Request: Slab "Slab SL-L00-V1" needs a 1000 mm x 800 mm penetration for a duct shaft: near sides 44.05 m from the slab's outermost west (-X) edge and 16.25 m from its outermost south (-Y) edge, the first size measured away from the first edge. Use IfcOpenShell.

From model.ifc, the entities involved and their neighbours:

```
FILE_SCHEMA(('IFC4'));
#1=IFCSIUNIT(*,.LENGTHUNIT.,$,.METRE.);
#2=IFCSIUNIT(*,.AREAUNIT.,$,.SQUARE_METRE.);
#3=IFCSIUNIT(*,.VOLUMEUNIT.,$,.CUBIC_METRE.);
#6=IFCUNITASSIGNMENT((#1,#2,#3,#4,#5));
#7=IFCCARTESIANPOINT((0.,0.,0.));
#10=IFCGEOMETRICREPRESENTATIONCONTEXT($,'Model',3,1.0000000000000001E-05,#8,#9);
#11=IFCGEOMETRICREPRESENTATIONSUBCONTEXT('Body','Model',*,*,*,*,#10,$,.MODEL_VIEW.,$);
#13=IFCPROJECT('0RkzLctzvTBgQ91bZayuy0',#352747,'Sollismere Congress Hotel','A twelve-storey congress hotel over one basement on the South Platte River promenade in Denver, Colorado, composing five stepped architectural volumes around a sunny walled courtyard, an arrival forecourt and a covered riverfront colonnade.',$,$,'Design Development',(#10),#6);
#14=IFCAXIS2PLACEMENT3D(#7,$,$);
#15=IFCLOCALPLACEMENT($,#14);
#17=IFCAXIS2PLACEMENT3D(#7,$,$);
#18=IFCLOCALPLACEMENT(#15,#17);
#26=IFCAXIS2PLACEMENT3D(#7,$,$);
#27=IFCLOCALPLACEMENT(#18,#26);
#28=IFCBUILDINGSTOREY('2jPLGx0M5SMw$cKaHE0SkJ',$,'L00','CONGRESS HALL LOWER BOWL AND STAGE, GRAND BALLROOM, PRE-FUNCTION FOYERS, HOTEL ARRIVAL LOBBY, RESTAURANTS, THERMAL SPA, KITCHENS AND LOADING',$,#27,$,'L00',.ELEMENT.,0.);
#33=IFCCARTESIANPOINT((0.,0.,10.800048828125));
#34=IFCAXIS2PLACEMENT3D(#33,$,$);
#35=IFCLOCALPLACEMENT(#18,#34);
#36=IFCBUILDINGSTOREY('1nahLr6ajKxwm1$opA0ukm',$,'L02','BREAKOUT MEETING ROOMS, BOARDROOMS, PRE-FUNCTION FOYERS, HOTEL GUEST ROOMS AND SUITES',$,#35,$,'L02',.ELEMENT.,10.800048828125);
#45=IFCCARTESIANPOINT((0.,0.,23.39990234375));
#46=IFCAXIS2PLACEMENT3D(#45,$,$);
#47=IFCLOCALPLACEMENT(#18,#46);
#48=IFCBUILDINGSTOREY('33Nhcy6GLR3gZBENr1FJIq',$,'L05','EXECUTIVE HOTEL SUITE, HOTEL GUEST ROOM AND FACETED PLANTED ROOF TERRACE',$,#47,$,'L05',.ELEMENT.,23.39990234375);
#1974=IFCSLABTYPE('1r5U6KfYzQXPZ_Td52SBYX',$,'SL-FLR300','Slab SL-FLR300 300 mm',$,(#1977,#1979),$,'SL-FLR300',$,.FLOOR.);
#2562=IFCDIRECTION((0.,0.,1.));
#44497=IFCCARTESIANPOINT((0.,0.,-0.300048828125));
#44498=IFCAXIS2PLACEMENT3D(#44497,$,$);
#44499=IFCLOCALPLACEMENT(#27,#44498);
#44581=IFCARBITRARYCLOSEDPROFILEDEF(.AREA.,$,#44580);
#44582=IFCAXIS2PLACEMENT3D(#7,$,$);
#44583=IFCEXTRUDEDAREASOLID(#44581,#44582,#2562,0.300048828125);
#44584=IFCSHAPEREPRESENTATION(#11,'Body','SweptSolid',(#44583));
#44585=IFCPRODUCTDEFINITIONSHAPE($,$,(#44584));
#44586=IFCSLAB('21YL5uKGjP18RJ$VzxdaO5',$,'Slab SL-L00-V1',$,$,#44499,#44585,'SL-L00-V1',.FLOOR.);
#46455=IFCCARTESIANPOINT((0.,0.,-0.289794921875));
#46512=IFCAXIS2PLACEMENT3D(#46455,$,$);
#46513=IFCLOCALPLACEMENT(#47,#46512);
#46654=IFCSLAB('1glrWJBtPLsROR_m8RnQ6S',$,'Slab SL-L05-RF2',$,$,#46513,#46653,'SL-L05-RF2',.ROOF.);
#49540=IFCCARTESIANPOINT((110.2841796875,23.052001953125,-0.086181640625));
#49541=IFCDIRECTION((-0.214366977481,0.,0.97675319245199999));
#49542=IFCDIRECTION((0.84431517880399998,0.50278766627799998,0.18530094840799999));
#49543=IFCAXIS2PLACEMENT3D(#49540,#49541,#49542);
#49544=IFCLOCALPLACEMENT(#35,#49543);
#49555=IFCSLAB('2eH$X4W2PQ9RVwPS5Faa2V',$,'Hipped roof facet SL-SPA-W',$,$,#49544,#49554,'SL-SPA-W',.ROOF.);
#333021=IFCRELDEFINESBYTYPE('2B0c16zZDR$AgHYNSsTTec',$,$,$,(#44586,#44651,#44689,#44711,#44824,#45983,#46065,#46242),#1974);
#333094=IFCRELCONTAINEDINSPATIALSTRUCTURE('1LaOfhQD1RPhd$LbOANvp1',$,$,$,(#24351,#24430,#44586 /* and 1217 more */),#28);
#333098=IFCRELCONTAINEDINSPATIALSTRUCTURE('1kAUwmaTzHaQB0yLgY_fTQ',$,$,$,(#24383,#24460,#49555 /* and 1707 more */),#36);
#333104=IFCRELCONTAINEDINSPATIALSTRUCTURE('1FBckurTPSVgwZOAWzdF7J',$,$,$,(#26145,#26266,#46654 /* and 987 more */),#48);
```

```python
import numpy as np
import ifcopenshell
import ifcopenshell.api.feature
import ifcopenshell.api.geometry
import ifcopenshell.api.root
import ifcopenshell.geom
import ifcopenshell.util.placement
import ifcopenshell.util.representation
import ifcopenshell.util.shape
import ifcopenshell.util.unit

model = ifcopenshell.open("model.ifc")
unit_scale = ifcopenshell.util.unit.calculate_unit_scale(model)
settings = ifcopenshell.geom.settings()


def volume(element):
    """Net volume in cubic metres, openings subtracted."""
    shape = ifcopenshell.geom.create_shape(settings, element)
    return ifcopenshell.util.shape.get_volume(shape.geometry)


slab = model.by_guid("21YL5uKGjP18RJ$VzxdaO5")
before = volume(slab)

# Extent in the slab's own axes, in metres. The edges named are its -X and -Y sides.
slab_shape = ifcopenshell.geom.create_shape(settings, slab)
vertices = ifcopenshell.util.shape.get_vertices(slab_shape.geometry)
x_min, y_min, bottom = vertices.min(axis=0)
top = vertices[:, 2].max()

opening = ifcopenshell.api.root.create_entity(model, ifc_class="IfcOpeningElement", name="Duct shaft opening", predefined_type="OPENING")
context = ifcopenshell.util.representation.get_context(model, "Model", "Body", "MODEL_VIEW")
width, depth = 1, 0.8
outline = [(0.0, 0.0), (width, 0.0), (width, depth), (0.0, depth), (0.0, 0.0)]
# Overshoot both faces by 50 mm so the cut is clean.
shape = ifcopenshell.api.geometry.add_slab_representation(
    model, context=context, depth=top - bottom + 0.1, polyline=outline
)
ifcopenshell.api.geometry.assign_representation(model, product=opening, representation=shape)

matrix = ifcopenshell.util.placement.get_local_placement(slab.ObjectPlacement)
matrix[:, 3] = matrix @ np.append(np.array([x_min + 44.05, y_min + 16.25, bottom - 0.05]) / unit_scale, 1.0)
ifcopenshell.api.geometry.edit_object_placement(model, product=opening, matrix=matrix, is_si=False)
ifcopenshell.api.feature.add_feature(model, feature=opening, element=slab)

after = volume(slab)

print(f"slab volume {before:.3f} -> {after:.3f} m3")

model.write("model_v2.ifc")
```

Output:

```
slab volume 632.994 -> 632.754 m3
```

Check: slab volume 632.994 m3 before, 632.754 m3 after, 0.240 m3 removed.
